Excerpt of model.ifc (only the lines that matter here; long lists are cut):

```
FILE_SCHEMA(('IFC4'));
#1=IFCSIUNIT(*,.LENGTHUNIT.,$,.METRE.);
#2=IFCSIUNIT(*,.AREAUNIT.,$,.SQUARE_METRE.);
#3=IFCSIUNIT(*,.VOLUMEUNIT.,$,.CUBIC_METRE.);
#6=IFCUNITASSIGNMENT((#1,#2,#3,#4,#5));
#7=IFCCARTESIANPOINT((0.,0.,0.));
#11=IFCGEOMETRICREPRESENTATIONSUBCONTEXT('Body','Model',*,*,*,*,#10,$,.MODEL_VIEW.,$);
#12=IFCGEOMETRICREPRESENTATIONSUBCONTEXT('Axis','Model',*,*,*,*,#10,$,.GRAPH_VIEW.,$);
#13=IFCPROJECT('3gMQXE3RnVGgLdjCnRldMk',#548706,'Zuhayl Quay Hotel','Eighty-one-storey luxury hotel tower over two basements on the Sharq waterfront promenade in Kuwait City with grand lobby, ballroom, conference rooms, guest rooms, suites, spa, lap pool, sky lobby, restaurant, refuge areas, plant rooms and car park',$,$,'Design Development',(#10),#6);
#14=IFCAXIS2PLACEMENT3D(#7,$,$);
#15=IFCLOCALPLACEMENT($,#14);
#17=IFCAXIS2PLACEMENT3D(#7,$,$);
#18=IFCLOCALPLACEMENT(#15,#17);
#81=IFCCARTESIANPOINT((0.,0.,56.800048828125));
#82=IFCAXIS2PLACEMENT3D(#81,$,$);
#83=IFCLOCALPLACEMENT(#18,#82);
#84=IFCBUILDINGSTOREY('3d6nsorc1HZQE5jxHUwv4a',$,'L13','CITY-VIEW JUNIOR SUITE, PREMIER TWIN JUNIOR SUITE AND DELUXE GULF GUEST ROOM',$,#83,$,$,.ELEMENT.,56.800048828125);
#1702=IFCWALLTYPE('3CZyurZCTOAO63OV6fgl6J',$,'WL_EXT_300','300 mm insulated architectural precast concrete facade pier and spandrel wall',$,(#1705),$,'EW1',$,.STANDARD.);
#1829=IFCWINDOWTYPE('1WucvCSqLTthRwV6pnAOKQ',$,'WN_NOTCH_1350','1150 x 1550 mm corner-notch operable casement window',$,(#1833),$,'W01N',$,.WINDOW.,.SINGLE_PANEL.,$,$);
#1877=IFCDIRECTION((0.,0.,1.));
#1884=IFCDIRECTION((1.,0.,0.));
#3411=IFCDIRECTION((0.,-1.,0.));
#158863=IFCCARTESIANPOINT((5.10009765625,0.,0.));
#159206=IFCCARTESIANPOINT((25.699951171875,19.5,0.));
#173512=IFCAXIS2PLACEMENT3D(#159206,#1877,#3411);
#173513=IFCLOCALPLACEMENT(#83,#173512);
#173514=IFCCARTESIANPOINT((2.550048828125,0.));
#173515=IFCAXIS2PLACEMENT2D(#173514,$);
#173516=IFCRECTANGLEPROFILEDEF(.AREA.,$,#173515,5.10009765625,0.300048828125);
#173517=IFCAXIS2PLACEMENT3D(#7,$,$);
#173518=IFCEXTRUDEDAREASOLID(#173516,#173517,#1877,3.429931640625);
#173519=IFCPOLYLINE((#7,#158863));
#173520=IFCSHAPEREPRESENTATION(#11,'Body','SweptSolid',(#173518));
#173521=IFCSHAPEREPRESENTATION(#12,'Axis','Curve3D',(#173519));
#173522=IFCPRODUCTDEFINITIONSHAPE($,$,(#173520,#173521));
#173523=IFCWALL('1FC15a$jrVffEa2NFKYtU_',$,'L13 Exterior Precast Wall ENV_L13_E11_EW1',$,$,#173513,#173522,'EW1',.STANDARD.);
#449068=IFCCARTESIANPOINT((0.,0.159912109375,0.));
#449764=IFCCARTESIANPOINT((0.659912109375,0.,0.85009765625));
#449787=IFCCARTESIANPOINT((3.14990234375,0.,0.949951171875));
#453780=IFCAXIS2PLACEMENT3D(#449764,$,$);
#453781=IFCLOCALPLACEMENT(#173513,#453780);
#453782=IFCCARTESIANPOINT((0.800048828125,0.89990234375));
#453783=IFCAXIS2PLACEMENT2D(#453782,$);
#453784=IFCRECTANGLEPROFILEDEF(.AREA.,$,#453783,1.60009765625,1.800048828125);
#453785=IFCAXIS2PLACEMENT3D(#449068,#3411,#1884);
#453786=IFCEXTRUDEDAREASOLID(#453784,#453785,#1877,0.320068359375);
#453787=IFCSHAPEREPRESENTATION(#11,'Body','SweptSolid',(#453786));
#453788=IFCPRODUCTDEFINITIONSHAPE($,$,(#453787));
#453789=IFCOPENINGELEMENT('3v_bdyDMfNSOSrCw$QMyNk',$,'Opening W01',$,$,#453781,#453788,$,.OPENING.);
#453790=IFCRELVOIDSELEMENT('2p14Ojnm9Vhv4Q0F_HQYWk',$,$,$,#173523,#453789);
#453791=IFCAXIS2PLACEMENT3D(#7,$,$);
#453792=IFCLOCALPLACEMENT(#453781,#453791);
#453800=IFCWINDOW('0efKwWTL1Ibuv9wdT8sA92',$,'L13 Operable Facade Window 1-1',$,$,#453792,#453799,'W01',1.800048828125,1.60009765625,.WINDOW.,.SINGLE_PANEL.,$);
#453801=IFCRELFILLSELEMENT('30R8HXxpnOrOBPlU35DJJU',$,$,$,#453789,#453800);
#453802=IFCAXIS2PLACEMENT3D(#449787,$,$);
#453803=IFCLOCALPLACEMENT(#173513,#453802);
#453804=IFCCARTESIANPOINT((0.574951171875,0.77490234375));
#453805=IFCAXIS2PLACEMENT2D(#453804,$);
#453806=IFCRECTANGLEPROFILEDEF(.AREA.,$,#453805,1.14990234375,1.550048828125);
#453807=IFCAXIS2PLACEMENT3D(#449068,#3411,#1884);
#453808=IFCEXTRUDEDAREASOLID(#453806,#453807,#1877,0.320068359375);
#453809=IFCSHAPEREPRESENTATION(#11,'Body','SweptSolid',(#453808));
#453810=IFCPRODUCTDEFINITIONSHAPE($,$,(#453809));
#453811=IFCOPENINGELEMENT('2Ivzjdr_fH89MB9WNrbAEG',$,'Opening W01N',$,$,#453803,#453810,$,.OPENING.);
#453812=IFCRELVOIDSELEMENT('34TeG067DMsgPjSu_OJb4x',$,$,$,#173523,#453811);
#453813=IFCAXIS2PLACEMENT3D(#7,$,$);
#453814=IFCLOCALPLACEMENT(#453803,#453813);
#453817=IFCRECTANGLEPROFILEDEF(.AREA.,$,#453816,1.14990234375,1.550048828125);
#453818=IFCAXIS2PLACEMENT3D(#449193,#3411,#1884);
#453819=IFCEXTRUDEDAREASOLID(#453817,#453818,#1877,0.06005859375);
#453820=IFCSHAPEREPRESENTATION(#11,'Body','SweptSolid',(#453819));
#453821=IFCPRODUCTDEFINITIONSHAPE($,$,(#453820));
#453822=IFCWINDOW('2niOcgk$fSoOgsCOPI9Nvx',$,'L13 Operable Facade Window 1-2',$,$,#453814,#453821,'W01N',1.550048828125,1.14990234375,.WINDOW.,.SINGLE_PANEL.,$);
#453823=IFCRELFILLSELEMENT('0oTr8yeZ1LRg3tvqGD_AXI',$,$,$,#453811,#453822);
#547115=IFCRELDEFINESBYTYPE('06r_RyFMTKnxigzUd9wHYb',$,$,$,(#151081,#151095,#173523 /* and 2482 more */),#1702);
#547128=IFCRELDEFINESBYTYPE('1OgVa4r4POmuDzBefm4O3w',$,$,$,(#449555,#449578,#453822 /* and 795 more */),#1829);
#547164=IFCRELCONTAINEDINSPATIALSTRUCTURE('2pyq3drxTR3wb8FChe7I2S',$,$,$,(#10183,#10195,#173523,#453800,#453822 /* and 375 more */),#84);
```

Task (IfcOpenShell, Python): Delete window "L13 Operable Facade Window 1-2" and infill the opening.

```python
import ifcopenshell
import ifcopenshell.api.feature
import ifcopenshell.api.root
import ifcopenshell.geom
import ifcopenshell.util.shape

model = ifcopenshell.open("model.ifc")
settings = ifcopenshell.geom.settings()


def volume(element):
    """Net volume in cubic metres, openings subtracted."""
    shape = ifcopenshell.geom.create_shape(settings, element)
    return ifcopenshell.util.shape.get_volume(shape.geometry)


window = model.by_guid("2niOcgk$fSoOgsCOPI9Nvx")
opening = window.FillsVoids[0].RelatingOpeningElement
wall = opening.VoidsElements[0].RelatingBuildingElement
before = volume(wall)

ifcopenshell.api.root.remove_product(model, product=window)
ifcopenshell.api.feature.remove_feature(model, feature=opening)

after = volume(wall)

print(f"wall volume {before:.3f} -> {after:.3f} m3")

model.write("model_rev.ifc")
```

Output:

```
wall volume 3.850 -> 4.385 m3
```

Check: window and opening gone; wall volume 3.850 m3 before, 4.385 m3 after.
